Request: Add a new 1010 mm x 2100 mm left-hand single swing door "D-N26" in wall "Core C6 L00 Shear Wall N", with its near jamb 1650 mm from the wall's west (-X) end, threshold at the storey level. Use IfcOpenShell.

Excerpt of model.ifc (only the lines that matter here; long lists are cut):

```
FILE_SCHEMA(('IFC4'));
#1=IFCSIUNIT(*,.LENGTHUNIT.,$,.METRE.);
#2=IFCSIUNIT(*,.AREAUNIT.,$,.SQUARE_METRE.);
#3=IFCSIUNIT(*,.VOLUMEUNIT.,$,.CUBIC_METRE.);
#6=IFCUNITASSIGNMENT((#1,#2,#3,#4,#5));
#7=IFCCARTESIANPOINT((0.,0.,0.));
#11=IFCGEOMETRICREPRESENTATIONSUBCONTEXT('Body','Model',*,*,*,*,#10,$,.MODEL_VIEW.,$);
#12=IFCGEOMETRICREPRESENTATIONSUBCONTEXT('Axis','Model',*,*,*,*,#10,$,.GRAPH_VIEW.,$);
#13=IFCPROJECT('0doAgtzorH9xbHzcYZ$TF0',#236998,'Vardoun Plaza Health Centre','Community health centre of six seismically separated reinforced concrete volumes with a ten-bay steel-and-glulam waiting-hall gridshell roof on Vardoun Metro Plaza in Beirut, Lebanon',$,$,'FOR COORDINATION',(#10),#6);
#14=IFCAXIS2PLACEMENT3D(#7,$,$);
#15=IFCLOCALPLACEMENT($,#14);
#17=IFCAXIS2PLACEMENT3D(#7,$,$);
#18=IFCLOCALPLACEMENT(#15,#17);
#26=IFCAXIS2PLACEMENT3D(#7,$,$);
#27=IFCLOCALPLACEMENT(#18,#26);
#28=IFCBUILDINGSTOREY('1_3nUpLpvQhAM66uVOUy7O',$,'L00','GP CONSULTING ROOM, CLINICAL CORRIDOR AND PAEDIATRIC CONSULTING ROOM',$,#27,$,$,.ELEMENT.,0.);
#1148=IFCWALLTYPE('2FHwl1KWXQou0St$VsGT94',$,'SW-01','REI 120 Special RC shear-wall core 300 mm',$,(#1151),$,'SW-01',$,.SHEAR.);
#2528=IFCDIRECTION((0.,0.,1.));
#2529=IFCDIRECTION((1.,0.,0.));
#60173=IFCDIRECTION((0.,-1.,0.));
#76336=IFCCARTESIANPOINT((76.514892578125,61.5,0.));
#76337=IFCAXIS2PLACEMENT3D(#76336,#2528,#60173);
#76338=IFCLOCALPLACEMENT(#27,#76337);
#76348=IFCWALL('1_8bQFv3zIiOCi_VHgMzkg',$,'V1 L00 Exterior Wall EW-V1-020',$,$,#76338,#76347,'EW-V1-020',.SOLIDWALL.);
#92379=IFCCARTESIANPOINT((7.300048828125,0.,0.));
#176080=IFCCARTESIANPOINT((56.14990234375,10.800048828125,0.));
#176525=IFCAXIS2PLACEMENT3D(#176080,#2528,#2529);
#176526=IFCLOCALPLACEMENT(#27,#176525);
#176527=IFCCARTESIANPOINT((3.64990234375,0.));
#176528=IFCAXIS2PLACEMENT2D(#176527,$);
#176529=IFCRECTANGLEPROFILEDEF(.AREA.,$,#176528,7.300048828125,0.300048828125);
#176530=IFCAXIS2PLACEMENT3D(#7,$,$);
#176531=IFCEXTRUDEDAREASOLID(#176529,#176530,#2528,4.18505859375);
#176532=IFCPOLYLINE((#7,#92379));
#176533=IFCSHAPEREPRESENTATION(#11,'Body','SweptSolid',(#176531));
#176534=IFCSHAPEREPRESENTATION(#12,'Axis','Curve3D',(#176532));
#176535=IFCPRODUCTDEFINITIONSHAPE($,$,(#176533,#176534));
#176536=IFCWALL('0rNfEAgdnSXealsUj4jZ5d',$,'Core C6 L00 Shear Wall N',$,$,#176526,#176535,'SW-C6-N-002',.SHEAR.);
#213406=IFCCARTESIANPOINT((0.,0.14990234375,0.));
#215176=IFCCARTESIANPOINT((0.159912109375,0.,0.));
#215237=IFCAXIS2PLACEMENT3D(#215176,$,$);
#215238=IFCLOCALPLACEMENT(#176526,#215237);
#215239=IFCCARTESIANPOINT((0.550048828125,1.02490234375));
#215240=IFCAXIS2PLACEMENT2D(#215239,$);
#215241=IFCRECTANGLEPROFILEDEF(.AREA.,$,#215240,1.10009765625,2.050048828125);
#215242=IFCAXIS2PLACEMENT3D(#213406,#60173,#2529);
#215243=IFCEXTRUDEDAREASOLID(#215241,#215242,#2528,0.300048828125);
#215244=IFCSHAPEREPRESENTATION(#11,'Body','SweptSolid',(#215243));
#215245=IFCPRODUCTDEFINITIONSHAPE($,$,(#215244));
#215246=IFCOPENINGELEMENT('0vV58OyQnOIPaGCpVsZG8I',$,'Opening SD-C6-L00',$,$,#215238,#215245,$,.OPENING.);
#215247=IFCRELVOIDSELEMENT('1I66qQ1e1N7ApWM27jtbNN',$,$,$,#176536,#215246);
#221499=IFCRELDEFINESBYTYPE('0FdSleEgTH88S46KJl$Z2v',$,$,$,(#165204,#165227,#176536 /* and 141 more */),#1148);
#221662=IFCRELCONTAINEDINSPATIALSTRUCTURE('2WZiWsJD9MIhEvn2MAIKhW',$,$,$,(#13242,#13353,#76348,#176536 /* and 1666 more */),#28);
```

```python
import numpy as np
import ifcopenshell
import ifcopenshell.api.feature
import ifcopenshell.api.geometry
import ifcopenshell.api.root
import ifcopenshell.api.spatial
import ifcopenshell.geom
import ifcopenshell.util.element
import ifcopenshell.util.placement
import ifcopenshell.util.representation
import ifcopenshell.util.shape
import ifcopenshell.util.unit

model = ifcopenshell.open("model.ifc")
unit_scale = ifcopenshell.util.unit.calculate_unit_scale(model)
settings = ifcopenshell.geom.settings()


def volume(element):
    """Net volume in cubic metres, openings subtracted."""
    shape = ifcopenshell.geom.create_shape(settings, element)
    return ifcopenshell.util.shape.get_volume(shape.geometry)


wall = model.by_guid("0rNfEAgdnSXealsUj4jZ5d")
storey = ifcopenshell.util.element.get_container(wall, ifc_class="IfcBuildingStorey")
context = ifcopenshell.util.representation.get_context(model, "Model", "Body", "MODEL_VIEW")
before = volume(wall)

width, height, from_end, sill = 1.01, 2.1, 1.65, 0.0  # metres

# The wall runs along its own X axis, and the end named is its -X end.
wall_shape = ifcopenshell.geom.create_shape(settings, wall)
x, y, z = ifcopenshell.util.shape.get_vertices(wall_shape.geometry).T
start = x.min() + from_end
face, thickness = float(y.min()), float(y.max() - y.min())
wall_matrix = ifcopenshell.util.placement.get_local_placement(wall.ObjectPlacement)
level = ifcopenshell.util.placement.get_local_placement(storey.ObjectPlacement)[2, 3]


def in_wall(x, y):
    """Placement at x, y metres in the wall's axes, at sill height."""
    matrix = wall_matrix.copy()
    matrix[:, 3] = wall_matrix @ np.array([x / unit_scale, y / unit_scale, 0.0, 1.0])
    matrix[2, 3] = level + sill / unit_scale
    return matrix


# Opening: a box that overshoots both wall faces by 50 mm.
opening = ifcopenshell.api.root.create_entity(model, ifc_class="IfcOpeningElement", predefined_type="OPENING")
box = ifcopenshell.api.geometry.add_wall_representation(
    model, context=context, length=width, height=height, thickness=thickness + 0.1
)
ifcopenshell.api.geometry.assign_representation(model, product=opening, representation=box)
ifcopenshell.api.geometry.edit_object_placement(model, product=opening, matrix=in_wall(start, face - 0.05), is_si=False)
ifcopenshell.api.feature.add_feature(model, feature=opening, element=wall)

door = ifcopenshell.api.root.create_entity(model, ifc_class="IfcDoor", name="D-N26", predefined_type="DOOR")
door.OverallWidth, door.OverallHeight = width / unit_scale, height / unit_scale
door.OperationType = "SINGLE_SWING_LEFT"
body = ifcopenshell.api.geometry.add_door_representation(
    model,
    context=context,
    overall_width=door.OverallWidth,
    overall_height=door.OverallHeight,
    operation_type="SINGLE_SWING_LEFT",
    lining_properties={"LiningDepth": thickness / unit_scale, "ThresholdDepth": thickness / unit_scale},
)
ifcopenshell.api.geometry.assign_representation(model, product=door, representation=body)
ifcopenshell.api.spatial.assign_container(model, products=[door], relating_structure=storey)
ifcopenshell.api.feature.add_filling(model, opening=opening, element=door)

# The lining spans the wall, so the door starts at the wall face.
ifcopenshell.api.geometry.edit_object_placement(model, product=door, matrix=in_wall(start, face), is_si=False)

after = volume(wall)

print(f"wall volume {before:.3f} -> {after:.3f} m3")

model.write("model_rev.ifc")
```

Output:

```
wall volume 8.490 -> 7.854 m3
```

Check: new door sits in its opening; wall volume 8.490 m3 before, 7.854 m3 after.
